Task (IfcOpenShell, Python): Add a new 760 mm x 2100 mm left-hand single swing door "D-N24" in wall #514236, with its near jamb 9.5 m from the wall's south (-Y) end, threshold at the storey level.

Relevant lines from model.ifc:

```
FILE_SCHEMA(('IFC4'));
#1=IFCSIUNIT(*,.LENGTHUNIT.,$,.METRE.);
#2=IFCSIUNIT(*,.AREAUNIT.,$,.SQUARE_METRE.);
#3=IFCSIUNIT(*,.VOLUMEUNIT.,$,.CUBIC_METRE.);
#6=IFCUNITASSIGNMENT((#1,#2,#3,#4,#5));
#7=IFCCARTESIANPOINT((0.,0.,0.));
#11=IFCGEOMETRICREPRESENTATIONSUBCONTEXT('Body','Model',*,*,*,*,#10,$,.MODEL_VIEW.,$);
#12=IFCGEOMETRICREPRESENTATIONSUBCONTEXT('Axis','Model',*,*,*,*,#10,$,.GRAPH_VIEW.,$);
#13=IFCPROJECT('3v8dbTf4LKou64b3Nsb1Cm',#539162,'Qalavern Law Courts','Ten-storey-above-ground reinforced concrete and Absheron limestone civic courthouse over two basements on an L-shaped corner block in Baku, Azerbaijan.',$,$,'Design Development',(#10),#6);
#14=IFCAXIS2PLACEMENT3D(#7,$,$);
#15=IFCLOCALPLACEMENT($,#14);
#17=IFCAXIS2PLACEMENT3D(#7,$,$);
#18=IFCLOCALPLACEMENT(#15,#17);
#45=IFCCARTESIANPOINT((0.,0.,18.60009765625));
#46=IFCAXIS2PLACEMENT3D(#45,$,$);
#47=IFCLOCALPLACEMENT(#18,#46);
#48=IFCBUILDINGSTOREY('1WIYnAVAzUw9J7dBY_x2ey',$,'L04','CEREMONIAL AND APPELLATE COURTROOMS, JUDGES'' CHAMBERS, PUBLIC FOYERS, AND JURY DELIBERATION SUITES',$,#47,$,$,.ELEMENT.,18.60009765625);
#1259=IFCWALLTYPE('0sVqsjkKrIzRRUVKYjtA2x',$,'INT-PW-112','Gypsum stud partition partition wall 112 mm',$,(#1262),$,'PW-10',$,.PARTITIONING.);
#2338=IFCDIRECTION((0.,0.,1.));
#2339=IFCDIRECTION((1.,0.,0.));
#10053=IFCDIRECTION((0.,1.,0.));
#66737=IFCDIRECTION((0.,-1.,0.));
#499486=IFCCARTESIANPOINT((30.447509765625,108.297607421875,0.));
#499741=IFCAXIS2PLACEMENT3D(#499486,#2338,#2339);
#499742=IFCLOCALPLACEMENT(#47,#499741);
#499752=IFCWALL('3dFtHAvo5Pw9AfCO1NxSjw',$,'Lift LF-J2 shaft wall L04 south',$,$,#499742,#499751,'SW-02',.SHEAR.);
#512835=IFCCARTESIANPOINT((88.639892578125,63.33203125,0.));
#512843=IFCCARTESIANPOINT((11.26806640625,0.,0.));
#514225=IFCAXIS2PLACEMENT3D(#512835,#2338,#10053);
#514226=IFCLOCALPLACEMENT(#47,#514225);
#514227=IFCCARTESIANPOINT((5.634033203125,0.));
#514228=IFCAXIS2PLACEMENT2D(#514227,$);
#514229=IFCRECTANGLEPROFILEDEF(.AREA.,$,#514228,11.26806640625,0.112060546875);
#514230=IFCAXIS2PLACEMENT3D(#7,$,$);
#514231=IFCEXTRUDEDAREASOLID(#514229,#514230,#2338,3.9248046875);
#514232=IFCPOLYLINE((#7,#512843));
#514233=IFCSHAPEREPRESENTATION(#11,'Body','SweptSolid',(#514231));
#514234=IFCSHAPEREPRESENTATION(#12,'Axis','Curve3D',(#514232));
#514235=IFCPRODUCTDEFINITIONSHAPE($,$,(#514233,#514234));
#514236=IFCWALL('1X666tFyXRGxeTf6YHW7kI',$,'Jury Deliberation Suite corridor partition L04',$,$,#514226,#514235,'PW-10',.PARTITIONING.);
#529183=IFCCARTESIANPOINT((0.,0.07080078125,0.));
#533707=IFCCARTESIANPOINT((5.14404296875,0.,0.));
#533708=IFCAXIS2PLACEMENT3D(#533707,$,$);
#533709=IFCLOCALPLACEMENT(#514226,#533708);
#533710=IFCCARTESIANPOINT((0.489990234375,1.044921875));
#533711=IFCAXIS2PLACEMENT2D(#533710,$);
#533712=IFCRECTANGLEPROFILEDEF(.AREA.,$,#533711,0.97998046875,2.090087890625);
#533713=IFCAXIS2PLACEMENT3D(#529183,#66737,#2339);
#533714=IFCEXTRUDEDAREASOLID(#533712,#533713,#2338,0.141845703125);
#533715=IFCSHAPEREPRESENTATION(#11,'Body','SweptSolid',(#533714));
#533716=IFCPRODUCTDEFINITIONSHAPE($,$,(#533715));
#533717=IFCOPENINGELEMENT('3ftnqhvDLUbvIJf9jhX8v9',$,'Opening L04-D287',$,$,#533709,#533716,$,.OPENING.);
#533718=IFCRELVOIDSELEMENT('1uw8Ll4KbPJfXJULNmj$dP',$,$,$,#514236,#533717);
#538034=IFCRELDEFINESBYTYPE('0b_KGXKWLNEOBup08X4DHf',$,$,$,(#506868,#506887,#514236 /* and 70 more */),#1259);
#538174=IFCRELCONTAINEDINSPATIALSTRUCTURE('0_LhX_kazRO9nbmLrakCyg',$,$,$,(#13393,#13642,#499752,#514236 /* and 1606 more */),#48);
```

```python
import numpy as np
import ifcopenshell
import ifcopenshell.api.feature
import ifcopenshell.api.geometry
import ifcopenshell.api.root
import ifcopenshell.api.spatial
import ifcopenshell.geom
import ifcopenshell.util.element
import ifcopenshell.util.placement
import ifcopenshell.util.representation
import ifcopenshell.util.shape
import ifcopenshell.util.unit

model = ifcopenshell.open("model.ifc")
unit_scale = ifcopenshell.util.unit.calculate_unit_scale(model)
settings = ifcopenshell.geom.settings()


def volume(element):
    """Net volume in cubic metres, openings subtracted."""
    shape = ifcopenshell.geom.create_shape(settings, element)
    return ifcopenshell.util.shape.get_volume(shape.geometry)


wall = model.by_guid("1X666tFyXRGxeTf6YHW7kI")
storey = ifcopenshell.util.element.get_container(wall, ifc_class="IfcBuildingStorey")
context = ifcopenshell.util.representation.get_context(model, "Model", "Body", "MODEL_VIEW")
before = volume(wall)

width, height, from_end, sill = 0.76, 2.1, 9.5, 0.0  # metres

# The wall runs along its own X axis, and the end named is its -X end.
wall_shape = ifcopenshell.geom.create_shape(settings, wall)
x, y, z = ifcopenshell.util.shape.get_vertices(wall_shape.geometry).T
start = x.min() + from_end
face, thickness = float(y.min()), float(y.max() - y.min())
wall_matrix = ifcopenshell.util.placement.get_local_placement(wall.ObjectPlacement)
level = ifcopenshell.util.placement.get_local_placement(storey.ObjectPlacement)[2, 3]


def in_wall(x, y):
    """Placement at x, y metres in the wall's axes, at sill height."""
    matrix = wall_matrix.copy()
    matrix[:, 3] = wall_matrix @ np.array([x / unit_scale, y / unit_scale, 0.0, 1.0])
    matrix[2, 3] = level + sill / unit_scale
    return matrix


# Opening: a box that overshoots both wall faces by 50 mm.
opening = ifcopenshell.api.root.create_entity(model, ifc_class="IfcOpeningElement", predefined_type="OPENING")
box = ifcopenshell.api.geometry.add_wall_representation(
    model, context=context, length=width, height=height, thickness=thickness + 0.1
)
ifcopenshell.api.geometry.assign_representation(model, product=opening, representation=box)
ifcopenshell.api.geometry.edit_object_placement(model, product=opening, matrix=in_wall(start, face - 0.05), is_si=False)
ifcopenshell.api.feature.add_feature(model, feature=opening, element=wall)

door = ifcopenshell.api.root.create_entity(model, ifc_class="IfcDoor", name="D-N24", predefined_type="DOOR")
door.OverallWidth, door.OverallHeight = width / unit_scale, height / unit_scale
door.OperationType = "SINGLE_SWING_LEFT"
body = ifcopenshell.api.geometry.add_door_representation(
    model,
    context=context,
    overall_width=door.OverallWidth,
    overall_height=door.OverallHeight,
    operation_type="SINGLE_SWING_LEFT",
    lining_properties={"LiningDepth": thickness / unit_scale, "ThresholdDepth": thickness / unit_scale},
)
ifcopenshell.api.geometry.assign_representation(model, product=door, representation=body)
ifcopenshell.api.spatial.assign_container(model, products=[door], relating_structure=storey)
ifcopenshell.api.feature.add_filling(model, opening=opening, element=door)

# The lining spans the wall, so the door starts at the wall face.
ifcopenshell.api.geometry.edit_object_placement(model, product=door, matrix=in_wall(start, face), is_si=False)

after = volume(wall)

print(f"wall volume {before:.3f} -> {after:.3f} m3")

model.write("model-out.ifc")
```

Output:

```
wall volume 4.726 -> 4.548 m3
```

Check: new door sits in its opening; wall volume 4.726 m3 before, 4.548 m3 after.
